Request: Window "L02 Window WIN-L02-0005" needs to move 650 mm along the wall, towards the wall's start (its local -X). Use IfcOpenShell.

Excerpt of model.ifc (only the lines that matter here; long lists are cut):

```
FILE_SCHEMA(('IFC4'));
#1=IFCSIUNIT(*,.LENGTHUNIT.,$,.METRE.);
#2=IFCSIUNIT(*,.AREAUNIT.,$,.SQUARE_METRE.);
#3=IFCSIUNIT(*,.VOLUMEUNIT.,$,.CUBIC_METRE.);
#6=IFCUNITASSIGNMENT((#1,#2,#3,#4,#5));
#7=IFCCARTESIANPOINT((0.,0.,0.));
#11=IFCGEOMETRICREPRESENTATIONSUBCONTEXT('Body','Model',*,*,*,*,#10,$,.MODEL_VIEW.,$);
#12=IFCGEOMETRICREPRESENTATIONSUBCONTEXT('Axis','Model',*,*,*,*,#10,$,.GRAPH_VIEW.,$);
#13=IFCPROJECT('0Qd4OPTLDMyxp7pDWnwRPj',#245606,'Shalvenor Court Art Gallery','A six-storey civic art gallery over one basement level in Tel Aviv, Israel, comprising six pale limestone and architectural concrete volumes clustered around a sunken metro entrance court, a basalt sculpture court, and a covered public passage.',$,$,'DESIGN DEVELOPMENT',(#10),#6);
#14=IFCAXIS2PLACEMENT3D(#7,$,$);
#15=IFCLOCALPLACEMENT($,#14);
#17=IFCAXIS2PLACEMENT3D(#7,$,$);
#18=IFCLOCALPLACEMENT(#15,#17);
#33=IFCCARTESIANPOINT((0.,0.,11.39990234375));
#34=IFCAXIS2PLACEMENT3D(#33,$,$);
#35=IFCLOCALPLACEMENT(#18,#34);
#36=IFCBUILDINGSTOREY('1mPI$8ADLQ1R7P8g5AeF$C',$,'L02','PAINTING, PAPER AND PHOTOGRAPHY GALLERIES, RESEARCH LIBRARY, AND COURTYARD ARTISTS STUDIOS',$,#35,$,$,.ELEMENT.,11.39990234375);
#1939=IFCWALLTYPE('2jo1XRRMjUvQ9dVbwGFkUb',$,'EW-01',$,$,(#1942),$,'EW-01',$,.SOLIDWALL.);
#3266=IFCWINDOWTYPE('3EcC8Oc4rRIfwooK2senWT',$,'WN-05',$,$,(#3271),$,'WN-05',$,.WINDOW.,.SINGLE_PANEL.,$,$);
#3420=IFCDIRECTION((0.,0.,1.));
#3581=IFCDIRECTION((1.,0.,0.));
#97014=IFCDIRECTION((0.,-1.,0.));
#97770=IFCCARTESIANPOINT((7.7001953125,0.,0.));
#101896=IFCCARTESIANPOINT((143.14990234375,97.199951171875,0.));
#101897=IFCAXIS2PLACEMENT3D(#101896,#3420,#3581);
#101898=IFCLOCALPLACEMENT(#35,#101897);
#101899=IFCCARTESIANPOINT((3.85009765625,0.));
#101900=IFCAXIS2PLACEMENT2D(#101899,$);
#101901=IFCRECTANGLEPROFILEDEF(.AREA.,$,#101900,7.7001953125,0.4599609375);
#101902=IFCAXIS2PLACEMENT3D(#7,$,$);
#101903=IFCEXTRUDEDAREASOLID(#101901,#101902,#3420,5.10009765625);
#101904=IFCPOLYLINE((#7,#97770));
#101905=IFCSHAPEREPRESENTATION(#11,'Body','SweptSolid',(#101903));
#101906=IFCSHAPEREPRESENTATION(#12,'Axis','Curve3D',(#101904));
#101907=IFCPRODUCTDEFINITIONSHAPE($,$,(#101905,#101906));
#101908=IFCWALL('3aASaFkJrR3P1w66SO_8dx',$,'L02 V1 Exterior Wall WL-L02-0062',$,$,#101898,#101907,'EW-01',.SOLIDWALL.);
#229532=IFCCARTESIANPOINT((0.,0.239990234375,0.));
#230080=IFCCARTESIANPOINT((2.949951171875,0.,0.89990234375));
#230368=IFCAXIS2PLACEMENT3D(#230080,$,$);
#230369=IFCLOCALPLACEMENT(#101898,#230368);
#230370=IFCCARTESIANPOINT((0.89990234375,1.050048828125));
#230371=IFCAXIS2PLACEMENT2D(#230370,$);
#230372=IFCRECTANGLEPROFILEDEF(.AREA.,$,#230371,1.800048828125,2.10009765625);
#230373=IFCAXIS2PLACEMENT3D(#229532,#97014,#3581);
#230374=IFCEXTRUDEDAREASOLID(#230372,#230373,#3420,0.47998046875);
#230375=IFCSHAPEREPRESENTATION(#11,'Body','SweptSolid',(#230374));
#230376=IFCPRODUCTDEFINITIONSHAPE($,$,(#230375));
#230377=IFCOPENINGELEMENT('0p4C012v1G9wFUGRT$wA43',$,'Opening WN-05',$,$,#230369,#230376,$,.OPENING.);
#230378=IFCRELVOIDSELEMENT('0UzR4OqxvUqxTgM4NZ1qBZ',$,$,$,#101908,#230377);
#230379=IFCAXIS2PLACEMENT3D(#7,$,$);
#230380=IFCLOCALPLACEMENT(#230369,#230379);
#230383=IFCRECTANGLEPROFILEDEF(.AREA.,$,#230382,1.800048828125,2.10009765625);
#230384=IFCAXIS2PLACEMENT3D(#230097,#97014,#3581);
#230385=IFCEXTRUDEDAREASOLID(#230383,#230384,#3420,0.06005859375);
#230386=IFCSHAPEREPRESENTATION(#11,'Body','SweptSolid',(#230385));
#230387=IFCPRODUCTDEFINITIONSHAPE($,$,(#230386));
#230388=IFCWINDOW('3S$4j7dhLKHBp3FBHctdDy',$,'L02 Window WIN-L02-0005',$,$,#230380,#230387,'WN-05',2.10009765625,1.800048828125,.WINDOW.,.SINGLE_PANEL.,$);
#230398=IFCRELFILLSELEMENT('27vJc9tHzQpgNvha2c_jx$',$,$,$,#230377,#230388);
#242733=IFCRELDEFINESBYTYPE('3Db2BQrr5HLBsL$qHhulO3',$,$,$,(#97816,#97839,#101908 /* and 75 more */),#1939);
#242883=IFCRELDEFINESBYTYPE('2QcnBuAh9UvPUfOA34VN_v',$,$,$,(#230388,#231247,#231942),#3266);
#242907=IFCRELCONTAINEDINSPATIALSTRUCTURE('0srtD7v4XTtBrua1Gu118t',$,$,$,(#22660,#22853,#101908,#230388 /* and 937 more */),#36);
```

```python
import ifcopenshell
import ifcopenshell.api.geometry
import ifcopenshell.util.placement

model = ifcopenshell.open("model.ifc")

window = model.by_guid("3S$4j7dhLKHBp3FBHctdDy")
opening = window.FillsVoids[0].RelatingOpeningElement
wall = opening.VoidsElements[0].RelatingBuildingElement

wall_matrix = ifcopenshell.util.placement.get_local_placement(wall.ObjectPlacement)
shift = wall_matrix[:3, 0] * -0.65
before = ifcopenshell.util.placement.get_local_placement(window.ObjectPlacement)[:3, 3].copy()

# The window is placed relative to its opening, so it follows when the opening moves.
matrix = ifcopenshell.util.placement.get_local_placement(opening.ObjectPlacement)
matrix[:3, 3] += shift
ifcopenshell.api.geometry.edit_object_placement(
    model, product=opening, matrix=matrix, is_si=False, should_transform_children=True
)

after = ifcopenshell.util.placement.get_local_placement(window.ObjectPlacement)[:3, 3]
print("window moved by", (after - before).round(3) + 0.0)

model.write("model_updated.ifc")
```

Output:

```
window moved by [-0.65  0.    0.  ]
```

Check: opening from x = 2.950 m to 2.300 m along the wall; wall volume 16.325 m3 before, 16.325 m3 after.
